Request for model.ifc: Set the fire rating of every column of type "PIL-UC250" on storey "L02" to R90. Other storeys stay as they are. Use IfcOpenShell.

First a look at what the model holds.

```python
import ifcopenshell
import ifcopenshell.util.element

model = ifcopenshell.open("model.ifc")
print(model.schema)
storey = next(s for s in model.by_type("IfcBuildingStorey") if s.Name == "L02")
columns = [e for e in ifcopenshell.util.element.get_decomposition(storey) if e.is_a("IfcColumn")]
seen = {}
for e in columns:
    element_type = ifcopenshell.util.element.get_type(e)
    key = (element_type.Name if element_type != e and element_type else None, ifcopenshell.util.element.get_pset(e, "Pset_ColumnCommon", "FireRating"))
    seen[key] = seen.get(key, 0) + 1
for (name, value), count in sorted(seen.items(), key=str):
    print(count, "x", name, "|", value)
```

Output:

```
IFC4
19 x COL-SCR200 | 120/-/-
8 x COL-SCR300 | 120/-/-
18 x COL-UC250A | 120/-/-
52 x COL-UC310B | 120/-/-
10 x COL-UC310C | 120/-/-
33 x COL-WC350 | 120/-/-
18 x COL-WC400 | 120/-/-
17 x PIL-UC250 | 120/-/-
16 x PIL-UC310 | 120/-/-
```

```python
import ifcopenshell
import ifcopenshell.api.pset
import ifcopenshell.util.element

model = ifcopenshell.open("model.ifc")

storey = next(s for s in model.by_type("IfcBuildingStorey") if s.Name == "L02")
columns = [e for e in ifcopenshell.util.element.get_decomposition(storey) if e.is_a("IfcColumn")]

count = 0
for e in columns:
    element_type = ifcopenshell.util.element.get_type(e)
    if element_type in (None, e) or element_type.Name != "PIL-UC250":
        continue
    # add_pset returns the element's existing set when there is one.
    pset = ifcopenshell.api.pset.add_pset(model, product=e, name="Pset_ColumnCommon")
    ifcopenshell.api.pset.edit_pset(model, pset=pset, properties={"FireRating": "R90"})
    count += 1

print(count, "columns updated")

model.write("model_edited.ifc")
```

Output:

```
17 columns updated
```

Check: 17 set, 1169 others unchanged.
